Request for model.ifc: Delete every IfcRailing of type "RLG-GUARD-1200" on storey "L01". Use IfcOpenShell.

First a look at what the model holds.

```python
import ifcopenshell
import ifcopenshell.util.element

model = ifcopenshell.open("model.ifc")
print(model.schema)
storey = next(s for s in model.by_type("IfcBuildingStorey") if s.Name == "L01")
railings = [e for e in ifcopenshell.util.element.get_decomposition(storey) if e.is_a("IfcRailing")]
seen = {}
for e in railings:
    element_type = ifcopenshell.util.element.get_type(e)
    name = element_type.Name if element_type not in (None, e) else None
    seen[name] = seen.get(name, 0) + 1
for name, count in sorted(seen.items(), key=str):
    print(count, "x", name)
```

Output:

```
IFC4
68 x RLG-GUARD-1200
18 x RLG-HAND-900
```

```python
import ifcopenshell
import ifcopenshell.api.root
import ifcopenshell.util.element

model = ifcopenshell.open("model.ifc")

storey = next(s for s in model.by_type("IfcBuildingStorey") if s.Name == "L01")
railings = [e for e in ifcopenshell.util.element.get_decomposition(storey) if e.is_a("IfcRailing")]
targets = [e for e in railings if (t := ifcopenshell.util.element.get_type(e)) not in (None, e) and t.Name == "RLG-GUARD-1200"]

for e in targets:
    ifcopenshell.api.root.remove_product(model, product=e)
print(len(targets), "removed")

model.write("model_updated.ifc")
```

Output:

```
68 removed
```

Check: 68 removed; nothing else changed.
